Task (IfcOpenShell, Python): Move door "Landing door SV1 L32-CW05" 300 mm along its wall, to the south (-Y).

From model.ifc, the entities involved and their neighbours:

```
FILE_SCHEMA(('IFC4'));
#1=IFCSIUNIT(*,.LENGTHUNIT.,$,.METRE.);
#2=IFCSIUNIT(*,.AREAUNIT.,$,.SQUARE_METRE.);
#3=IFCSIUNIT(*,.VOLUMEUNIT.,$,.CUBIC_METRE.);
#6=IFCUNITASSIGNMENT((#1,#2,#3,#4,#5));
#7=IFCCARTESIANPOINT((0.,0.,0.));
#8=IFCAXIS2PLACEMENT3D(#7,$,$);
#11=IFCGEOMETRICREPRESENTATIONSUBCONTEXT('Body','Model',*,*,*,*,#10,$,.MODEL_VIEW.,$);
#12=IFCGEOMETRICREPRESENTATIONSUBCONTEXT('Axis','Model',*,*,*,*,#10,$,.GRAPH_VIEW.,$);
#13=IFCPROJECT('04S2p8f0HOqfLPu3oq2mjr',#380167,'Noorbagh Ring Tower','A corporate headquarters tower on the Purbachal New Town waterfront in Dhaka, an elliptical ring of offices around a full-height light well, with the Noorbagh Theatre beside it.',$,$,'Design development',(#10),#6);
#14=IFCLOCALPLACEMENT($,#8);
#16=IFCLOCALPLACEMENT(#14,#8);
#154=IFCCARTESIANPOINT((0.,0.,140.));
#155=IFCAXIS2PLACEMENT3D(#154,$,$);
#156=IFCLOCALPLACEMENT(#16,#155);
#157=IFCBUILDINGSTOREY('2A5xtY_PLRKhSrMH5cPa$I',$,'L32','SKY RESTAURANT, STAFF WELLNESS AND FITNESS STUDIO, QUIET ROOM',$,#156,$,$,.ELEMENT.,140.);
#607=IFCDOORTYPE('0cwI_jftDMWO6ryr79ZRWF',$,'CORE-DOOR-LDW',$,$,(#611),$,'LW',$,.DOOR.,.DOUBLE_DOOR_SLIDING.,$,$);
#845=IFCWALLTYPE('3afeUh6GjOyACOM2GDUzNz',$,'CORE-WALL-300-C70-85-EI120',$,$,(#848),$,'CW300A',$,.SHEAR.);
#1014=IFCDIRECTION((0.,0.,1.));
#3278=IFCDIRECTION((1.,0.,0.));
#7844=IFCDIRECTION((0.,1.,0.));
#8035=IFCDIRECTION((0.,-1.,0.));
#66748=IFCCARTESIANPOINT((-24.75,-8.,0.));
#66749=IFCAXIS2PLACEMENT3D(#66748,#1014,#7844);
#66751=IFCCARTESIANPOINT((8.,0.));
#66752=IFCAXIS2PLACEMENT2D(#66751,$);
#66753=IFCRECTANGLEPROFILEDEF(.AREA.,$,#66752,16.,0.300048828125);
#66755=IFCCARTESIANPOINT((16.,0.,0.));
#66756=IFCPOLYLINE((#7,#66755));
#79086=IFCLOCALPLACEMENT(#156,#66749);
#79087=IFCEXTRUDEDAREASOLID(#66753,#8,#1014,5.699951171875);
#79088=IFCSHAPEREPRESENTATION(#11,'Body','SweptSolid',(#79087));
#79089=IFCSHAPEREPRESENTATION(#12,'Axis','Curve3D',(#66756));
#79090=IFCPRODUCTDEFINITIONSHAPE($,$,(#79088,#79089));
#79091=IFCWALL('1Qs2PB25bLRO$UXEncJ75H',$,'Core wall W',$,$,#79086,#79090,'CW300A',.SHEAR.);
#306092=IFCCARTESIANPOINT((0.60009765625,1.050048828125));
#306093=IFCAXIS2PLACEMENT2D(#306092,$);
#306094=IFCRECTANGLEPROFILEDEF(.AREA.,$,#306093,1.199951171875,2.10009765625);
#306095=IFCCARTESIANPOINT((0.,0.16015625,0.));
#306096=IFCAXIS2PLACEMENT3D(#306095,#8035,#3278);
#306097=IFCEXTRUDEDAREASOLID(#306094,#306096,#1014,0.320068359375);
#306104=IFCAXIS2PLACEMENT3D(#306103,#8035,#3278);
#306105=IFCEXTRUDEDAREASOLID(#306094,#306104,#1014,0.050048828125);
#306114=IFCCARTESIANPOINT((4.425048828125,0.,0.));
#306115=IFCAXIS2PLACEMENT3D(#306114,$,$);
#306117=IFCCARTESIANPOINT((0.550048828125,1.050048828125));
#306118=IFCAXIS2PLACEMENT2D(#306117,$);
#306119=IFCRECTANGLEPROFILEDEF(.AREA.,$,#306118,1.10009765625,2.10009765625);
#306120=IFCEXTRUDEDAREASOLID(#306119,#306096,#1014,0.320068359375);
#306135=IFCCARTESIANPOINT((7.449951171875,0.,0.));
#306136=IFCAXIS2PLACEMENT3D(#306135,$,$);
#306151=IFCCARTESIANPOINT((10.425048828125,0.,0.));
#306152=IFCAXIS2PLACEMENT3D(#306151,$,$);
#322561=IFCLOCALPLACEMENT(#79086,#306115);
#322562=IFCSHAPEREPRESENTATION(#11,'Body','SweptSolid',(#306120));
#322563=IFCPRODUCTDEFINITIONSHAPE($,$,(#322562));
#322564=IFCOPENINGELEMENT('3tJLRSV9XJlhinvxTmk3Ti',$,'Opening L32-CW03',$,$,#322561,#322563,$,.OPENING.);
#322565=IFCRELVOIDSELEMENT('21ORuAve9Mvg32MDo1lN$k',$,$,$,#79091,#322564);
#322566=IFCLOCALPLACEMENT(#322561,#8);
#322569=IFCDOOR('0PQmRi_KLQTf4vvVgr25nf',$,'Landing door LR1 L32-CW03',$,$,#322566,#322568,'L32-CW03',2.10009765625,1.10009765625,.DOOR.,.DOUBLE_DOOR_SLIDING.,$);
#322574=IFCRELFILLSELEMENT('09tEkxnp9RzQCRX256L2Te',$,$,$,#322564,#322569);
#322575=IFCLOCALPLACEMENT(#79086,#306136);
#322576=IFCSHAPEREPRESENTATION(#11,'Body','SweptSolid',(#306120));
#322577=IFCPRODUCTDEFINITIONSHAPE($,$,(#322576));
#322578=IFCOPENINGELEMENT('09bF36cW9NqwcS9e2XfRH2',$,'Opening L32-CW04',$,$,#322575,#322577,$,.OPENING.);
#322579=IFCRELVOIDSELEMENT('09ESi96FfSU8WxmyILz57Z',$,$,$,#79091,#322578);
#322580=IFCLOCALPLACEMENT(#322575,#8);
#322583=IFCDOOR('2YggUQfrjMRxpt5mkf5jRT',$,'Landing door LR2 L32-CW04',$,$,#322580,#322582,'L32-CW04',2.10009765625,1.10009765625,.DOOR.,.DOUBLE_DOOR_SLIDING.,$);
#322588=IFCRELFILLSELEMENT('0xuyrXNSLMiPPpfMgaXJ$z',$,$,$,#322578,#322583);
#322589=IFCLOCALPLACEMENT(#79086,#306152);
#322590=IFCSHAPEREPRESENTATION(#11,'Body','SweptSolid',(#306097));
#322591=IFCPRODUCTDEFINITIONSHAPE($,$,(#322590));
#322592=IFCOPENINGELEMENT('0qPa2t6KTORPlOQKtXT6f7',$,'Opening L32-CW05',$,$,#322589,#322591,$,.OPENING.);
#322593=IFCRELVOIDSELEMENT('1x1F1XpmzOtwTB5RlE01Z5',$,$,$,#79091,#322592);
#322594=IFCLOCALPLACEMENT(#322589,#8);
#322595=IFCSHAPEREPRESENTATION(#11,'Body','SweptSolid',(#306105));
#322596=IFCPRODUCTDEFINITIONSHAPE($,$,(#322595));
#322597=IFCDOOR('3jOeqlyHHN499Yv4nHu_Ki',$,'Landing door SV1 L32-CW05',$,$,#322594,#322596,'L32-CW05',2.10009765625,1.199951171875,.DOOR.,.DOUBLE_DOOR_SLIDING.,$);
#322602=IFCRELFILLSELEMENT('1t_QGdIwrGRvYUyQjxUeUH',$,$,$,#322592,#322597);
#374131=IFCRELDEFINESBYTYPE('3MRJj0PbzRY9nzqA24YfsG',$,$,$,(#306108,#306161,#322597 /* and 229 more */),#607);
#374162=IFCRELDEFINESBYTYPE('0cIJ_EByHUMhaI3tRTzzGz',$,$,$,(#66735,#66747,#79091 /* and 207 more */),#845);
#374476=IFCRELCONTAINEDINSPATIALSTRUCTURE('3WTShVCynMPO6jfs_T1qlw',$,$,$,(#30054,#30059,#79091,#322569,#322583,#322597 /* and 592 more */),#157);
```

```python
import ifcopenshell
import ifcopenshell.api.geometry
import ifcopenshell.util.placement
import ifcopenshell.util.unit

model = ifcopenshell.open("model.ifc")
unit_scale = ifcopenshell.util.unit.calculate_unit_scale(model)

door = model.by_id(322597)
opening = door.FillsVoids[0].RelatingOpeningElement
wall = opening.VoidsElements[0].RelatingBuildingElement

wall_matrix = ifcopenshell.util.placement.get_local_placement(wall.ObjectPlacement)
shift = wall_matrix[:3, 0] * -0.3 / unit_scale
before = ifcopenshell.util.placement.get_local_placement(door.ObjectPlacement)[:3, 3].copy()

# The door is placed relative to its opening, so it follows when the opening moves.
matrix = ifcopenshell.util.placement.get_local_placement(opening.ObjectPlacement)
matrix[:3, 3] += shift
ifcopenshell.api.geometry.edit_object_placement(
    model, product=opening, matrix=matrix, is_si=False, should_transform_children=True
)

after = ifcopenshell.util.placement.get_local_placement(door.ObjectPlacement)[:3, 3]
print("door moved by", (after - before).round(3) + 0.0)

model.write("model_rev.ifc")
```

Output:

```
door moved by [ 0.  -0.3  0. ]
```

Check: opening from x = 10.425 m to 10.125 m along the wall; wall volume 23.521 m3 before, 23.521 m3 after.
